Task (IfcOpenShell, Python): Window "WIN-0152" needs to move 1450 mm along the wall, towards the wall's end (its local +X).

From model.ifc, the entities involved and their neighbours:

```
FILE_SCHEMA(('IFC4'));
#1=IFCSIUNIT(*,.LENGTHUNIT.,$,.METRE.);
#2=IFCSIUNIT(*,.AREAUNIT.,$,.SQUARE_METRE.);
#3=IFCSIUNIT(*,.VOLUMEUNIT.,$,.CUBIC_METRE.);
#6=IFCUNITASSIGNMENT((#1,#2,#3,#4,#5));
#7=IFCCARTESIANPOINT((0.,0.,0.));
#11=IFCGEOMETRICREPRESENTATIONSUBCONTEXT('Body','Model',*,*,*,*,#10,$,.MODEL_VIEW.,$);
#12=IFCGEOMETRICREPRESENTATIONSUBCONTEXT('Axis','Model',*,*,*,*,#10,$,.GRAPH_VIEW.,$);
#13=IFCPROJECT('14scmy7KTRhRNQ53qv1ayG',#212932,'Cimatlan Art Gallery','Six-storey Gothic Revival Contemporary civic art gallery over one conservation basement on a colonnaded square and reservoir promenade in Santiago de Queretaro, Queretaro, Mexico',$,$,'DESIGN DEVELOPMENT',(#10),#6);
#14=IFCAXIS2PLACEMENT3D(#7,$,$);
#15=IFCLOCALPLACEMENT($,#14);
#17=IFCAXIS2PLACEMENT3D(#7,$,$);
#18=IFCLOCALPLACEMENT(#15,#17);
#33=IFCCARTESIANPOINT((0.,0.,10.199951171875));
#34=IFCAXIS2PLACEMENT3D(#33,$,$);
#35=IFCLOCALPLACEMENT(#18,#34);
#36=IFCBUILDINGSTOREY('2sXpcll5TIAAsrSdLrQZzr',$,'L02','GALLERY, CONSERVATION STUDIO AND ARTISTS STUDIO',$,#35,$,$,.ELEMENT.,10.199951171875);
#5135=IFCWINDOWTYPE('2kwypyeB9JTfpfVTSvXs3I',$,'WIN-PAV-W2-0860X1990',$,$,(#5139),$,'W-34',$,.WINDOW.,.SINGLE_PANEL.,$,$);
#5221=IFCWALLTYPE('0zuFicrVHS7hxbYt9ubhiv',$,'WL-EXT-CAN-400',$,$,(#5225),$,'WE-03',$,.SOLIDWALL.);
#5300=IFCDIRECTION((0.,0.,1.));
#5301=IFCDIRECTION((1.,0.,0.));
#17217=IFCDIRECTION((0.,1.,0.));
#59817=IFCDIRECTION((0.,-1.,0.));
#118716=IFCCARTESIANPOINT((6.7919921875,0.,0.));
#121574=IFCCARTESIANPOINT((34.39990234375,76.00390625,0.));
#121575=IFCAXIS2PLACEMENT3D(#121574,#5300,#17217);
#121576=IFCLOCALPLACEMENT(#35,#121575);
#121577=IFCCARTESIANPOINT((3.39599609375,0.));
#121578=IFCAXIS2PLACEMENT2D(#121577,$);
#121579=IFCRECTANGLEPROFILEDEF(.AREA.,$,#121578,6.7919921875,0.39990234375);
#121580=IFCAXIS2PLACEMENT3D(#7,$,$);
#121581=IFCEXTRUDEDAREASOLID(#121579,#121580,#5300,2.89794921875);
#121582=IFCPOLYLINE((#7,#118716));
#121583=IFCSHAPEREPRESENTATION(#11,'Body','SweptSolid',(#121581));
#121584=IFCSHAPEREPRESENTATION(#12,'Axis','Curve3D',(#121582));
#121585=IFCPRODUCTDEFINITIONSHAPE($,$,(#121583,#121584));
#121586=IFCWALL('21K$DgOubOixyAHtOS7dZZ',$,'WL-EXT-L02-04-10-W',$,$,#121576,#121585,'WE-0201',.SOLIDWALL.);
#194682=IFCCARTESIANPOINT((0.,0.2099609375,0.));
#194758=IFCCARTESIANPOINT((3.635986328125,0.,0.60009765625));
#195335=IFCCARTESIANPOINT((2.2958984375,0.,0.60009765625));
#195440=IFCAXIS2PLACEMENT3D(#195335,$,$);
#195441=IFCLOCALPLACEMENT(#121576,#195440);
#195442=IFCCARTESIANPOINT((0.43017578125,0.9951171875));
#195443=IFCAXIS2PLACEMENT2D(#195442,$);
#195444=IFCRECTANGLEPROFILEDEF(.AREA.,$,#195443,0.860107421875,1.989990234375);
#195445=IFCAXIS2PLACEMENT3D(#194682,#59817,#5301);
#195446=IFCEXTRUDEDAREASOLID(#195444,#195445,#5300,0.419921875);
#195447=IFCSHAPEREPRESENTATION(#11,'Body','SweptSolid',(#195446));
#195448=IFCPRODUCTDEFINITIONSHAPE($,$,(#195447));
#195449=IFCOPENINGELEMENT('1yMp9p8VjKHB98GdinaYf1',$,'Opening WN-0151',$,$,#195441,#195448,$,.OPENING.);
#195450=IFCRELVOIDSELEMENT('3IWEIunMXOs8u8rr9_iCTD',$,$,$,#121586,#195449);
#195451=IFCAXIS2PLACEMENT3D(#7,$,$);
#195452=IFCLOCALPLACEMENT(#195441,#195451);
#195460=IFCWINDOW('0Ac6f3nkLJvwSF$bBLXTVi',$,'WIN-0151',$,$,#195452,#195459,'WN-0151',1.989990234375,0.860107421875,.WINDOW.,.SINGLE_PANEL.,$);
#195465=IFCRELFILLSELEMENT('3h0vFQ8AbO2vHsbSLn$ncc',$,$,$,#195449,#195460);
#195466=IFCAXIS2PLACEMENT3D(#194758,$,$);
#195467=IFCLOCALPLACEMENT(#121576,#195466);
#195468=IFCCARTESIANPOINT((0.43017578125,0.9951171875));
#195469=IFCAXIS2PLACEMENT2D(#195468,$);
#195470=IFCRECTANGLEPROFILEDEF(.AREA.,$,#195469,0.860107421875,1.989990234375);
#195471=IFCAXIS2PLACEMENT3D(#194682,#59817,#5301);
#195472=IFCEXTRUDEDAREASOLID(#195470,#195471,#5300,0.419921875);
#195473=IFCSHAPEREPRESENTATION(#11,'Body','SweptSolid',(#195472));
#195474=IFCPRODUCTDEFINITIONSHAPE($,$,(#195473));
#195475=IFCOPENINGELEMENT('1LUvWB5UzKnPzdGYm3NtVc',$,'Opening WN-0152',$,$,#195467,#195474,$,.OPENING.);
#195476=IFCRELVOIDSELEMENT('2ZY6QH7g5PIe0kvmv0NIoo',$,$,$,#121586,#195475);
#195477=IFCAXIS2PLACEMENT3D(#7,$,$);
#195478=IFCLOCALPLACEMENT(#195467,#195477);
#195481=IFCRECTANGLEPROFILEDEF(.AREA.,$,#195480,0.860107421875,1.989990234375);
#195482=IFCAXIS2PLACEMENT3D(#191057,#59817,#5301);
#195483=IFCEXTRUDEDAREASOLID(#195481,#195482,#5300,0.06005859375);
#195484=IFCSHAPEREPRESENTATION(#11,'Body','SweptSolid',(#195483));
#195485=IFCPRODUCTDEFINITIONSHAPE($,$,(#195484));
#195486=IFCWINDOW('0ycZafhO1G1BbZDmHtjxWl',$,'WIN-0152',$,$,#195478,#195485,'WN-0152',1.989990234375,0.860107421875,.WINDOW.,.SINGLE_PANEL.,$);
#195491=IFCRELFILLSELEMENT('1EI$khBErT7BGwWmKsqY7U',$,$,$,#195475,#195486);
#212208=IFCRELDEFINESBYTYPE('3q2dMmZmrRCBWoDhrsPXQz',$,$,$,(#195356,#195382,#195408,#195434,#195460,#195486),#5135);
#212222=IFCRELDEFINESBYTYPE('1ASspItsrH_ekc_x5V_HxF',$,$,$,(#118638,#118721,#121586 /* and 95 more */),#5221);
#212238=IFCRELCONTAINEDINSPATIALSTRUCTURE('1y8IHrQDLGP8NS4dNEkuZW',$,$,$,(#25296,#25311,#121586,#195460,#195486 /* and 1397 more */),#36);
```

```python
import ifcopenshell
import ifcopenshell.api.geometry
import ifcopenshell.util.placement
import ifcopenshell.util.unit

model = ifcopenshell.open("model.ifc")
unit_scale = ifcopenshell.util.unit.calculate_unit_scale(model)

window = model.by_id(195486)
opening = window.FillsVoids[0].RelatingOpeningElement
wall = opening.VoidsElements[0].RelatingBuildingElement

wall_matrix = ifcopenshell.util.placement.get_local_placement(wall.ObjectPlacement)
shift = wall_matrix[:3, 0] * 1.45 / unit_scale
before = ifcopenshell.util.placement.get_local_placement(window.ObjectPlacement)[:3, 3].copy()

# The window is placed relative to its opening, so it follows when the opening moves.
matrix = ifcopenshell.util.placement.get_local_placement(opening.ObjectPlacement)
matrix[:3, 3] += shift
ifcopenshell.api.geometry.edit_object_placement(
    model, product=opening, matrix=matrix, is_si=False, should_transform_children=True
)

after = ifcopenshell.util.placement.get_local_placement(window.ObjectPlacement)[:3, 3]
print("window moved by", (after - before).round(3) + 0.0)

model.write("model_edited.ifc")
```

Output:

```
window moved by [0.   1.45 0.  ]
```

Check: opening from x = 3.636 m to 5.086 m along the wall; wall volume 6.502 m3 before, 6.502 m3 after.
